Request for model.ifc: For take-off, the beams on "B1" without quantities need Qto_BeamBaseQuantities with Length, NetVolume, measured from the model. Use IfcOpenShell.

First a look at what the model holds.

```python
import ifcopenshell
import ifcopenshell.util.element
import ifcopenshell.util.unit

model = ifcopenshell.open("model.ifc")
print(model.schema)
for unit_type in ("LENGTHUNIT", "AREAUNIT", "VOLUMEUNIT"):
    print(unit_type, ifcopenshell.util.unit.calculate_unit_scale(model, unit_type))
storey = next(s for s in model.by_type("IfcBuildingStorey") if s.Name == "B1")
beams = [e for e in ifcopenshell.util.element.get_decomposition(storey) if e.is_a("IfcBeam")]
for e in sorted(beams, key=lambda e: e.id()):
    print(e.id(), e.is_a(), e.Name, list(ifcopenshell.util.element.get_psets(e, qtos_only=True)), sep=" | ")
```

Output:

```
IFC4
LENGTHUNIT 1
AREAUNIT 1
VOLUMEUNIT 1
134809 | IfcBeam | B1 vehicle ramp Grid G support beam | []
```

```python
import ifcopenshell
import ifcopenshell.api.pset
import ifcopenshell.geom
import ifcopenshell.util.element
import ifcopenshell.util.shape
import ifcopenshell.util.unit

model = ifcopenshell.open("model.ifc")
unit_scale = ifcopenshell.util.unit.calculate_unit_scale(model)
volume_scale = ifcopenshell.util.unit.calculate_unit_scale(model, "VOLUMEUNIT")
settings = ifcopenshell.geom.settings()

storey = next(s for s in model.by_type("IfcBuildingStorey") if s.Name == "B1")
beams = [e for e in ifcopenshell.util.element.get_decomposition(storey) if e.is_a("IfcBeam")]

for e in sorted(beams, key=lambda e: e.id()):
    if ifcopenshell.util.element.get_psets(e, qtos_only=True, should_inherit=False):
        continue
    # Geometry comes back in metres, in the element's own axes.
    shape = ifcopenshell.geom.create_shape(settings, e)
    values = {
        "Length": ifcopenshell.util.shape.get_max_xyz(shape.geometry) / unit_scale,
        "NetVolume": ifcopenshell.util.shape.get_volume(shape.geometry) / volume_scale,
    }
    qto = ifcopenshell.api.pset.add_qto(model, product=e, name="Qto_BeamBaseQuantities")
    ifcopenshell.api.pset.edit_qto(model, qto=qto, properties=values)
    print(e.id(), {k: round(v, 3) for k, v in values.items()})

model.write("model_v2.ifc")
```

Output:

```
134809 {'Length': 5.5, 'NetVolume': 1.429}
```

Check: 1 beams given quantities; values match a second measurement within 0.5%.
